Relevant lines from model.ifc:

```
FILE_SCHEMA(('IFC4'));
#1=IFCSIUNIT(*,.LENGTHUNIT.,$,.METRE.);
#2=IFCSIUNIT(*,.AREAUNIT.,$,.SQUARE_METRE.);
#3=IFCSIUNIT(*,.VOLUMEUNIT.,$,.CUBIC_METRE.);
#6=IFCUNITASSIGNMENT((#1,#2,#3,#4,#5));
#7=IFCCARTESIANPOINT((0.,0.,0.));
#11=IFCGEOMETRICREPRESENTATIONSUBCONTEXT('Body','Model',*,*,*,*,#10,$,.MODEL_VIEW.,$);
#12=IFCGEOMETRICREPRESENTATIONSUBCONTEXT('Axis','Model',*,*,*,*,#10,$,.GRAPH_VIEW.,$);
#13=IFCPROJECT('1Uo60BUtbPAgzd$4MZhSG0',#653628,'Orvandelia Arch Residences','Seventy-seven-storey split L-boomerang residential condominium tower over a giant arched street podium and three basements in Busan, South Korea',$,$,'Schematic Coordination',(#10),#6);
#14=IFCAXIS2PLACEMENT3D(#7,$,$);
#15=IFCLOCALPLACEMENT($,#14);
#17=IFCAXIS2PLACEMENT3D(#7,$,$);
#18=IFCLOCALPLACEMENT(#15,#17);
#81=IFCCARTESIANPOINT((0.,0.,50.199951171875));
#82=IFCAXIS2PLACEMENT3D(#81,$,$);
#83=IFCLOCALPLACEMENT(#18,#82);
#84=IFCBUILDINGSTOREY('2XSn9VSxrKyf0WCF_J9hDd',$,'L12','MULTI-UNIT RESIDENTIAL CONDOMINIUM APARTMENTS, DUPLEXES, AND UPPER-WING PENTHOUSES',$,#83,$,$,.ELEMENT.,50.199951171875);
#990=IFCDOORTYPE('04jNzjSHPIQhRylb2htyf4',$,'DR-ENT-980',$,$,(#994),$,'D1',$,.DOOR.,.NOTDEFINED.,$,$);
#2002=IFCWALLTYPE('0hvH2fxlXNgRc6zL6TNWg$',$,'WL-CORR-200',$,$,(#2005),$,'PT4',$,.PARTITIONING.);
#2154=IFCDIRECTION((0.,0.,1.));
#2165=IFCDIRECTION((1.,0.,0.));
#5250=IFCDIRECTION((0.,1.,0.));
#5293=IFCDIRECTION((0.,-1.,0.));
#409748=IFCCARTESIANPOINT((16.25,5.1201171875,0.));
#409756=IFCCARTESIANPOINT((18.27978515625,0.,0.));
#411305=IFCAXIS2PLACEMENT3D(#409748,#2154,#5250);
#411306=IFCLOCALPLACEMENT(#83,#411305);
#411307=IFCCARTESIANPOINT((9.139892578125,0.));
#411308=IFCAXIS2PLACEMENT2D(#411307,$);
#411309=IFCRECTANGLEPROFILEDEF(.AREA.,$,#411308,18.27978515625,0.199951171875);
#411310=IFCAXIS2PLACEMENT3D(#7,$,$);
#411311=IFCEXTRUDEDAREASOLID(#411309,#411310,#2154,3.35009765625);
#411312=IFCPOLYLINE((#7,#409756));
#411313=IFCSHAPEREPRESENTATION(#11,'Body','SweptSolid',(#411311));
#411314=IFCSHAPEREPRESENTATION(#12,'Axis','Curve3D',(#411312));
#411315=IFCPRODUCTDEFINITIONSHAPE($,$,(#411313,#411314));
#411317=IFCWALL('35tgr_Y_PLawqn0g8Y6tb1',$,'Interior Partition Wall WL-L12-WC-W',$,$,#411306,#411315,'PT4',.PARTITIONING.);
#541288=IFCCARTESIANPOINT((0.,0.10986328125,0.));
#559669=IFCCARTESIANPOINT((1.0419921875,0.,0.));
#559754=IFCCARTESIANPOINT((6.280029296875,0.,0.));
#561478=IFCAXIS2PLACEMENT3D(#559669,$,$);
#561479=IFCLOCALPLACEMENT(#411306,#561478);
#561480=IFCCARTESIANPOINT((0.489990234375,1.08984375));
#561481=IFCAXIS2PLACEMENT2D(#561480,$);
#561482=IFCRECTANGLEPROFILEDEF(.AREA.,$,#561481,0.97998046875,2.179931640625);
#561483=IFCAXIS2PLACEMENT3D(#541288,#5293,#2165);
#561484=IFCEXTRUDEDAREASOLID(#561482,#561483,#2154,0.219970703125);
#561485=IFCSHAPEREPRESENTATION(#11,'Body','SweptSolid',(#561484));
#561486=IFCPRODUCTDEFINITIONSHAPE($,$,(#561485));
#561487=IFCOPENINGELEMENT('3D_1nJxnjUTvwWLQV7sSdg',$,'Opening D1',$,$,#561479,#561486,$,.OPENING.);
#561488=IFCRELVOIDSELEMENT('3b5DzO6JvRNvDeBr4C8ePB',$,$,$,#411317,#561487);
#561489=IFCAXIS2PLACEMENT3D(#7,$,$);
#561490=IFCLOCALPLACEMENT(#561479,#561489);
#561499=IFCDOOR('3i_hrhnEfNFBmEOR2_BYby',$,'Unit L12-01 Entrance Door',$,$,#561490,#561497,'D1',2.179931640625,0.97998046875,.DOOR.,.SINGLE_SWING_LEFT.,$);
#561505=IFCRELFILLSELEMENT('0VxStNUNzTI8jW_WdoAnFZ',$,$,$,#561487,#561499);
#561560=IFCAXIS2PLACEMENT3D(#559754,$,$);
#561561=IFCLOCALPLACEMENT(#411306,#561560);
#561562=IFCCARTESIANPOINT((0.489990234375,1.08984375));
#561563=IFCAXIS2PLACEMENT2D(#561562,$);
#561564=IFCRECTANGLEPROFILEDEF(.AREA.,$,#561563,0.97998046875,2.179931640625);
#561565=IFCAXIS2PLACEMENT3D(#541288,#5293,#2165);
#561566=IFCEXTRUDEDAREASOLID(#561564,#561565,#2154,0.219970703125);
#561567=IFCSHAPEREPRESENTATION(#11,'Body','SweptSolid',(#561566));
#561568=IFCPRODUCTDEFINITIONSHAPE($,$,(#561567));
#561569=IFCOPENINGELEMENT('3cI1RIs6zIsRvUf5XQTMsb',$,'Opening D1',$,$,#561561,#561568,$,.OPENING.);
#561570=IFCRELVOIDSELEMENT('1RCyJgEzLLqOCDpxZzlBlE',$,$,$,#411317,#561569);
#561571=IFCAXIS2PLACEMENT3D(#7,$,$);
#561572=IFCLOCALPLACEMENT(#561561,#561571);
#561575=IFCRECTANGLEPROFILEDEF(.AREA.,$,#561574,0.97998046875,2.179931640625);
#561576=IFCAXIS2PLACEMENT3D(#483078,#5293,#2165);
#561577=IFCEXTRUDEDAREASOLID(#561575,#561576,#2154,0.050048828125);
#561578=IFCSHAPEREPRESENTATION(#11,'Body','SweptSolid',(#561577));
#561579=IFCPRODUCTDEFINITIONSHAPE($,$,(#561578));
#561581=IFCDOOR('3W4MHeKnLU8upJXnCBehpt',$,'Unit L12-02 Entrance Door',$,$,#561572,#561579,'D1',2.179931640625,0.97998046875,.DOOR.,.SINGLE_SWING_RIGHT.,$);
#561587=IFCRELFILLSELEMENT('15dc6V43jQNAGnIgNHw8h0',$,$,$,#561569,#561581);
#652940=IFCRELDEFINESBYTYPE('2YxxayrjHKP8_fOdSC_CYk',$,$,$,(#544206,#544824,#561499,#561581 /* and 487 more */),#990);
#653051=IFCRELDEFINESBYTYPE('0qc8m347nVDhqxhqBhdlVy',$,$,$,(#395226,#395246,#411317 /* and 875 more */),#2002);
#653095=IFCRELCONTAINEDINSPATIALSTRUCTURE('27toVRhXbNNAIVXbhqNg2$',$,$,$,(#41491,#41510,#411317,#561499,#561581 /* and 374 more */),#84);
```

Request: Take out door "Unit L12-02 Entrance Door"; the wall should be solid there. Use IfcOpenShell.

```python
import ifcopenshell
import ifcopenshell.api.feature
import ifcopenshell.api.root
import ifcopenshell.geom
import ifcopenshell.util.shape

model = ifcopenshell.open("model.ifc")
settings = ifcopenshell.geom.settings()


def volume(element):
    """Net volume in cubic metres, openings subtracted."""
    shape = ifcopenshell.geom.create_shape(settings, element)
    return ifcopenshell.util.shape.get_volume(shape.geometry)


door = model.by_guid("3W4MHeKnLU8upJXnCBehpt")
opening = door.FillsVoids[0].RelatingOpeningElement
wall = opening.VoidsElements[0].RelatingBuildingElement
before = volume(wall)

ifcopenshell.api.root.remove_product(model, product=door)
ifcopenshell.api.feature.remove_feature(model, feature=opening)

after = volume(wall)

print(f"wall volume {before:.3f} -> {after:.3f} m3")

model.write("model-out.ifc")
```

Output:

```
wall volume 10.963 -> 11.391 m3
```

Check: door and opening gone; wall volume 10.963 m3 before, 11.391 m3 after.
